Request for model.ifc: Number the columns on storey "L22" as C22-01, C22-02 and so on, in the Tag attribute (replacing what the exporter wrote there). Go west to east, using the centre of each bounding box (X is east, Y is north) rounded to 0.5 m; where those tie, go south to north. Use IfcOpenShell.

First a look at what the model holds.

```python
import ifcopenshell
import ifcopenshell.util.element
import ifcopenshell.util.placement

model = ifcopenshell.open("model.ifc")
print(model.schema)
storey = next(s for s in model.by_type("IfcBuildingStorey") if s.Name == "L22")
columns = [e for e in ifcopenshell.util.element.get_decomposition(storey) if e.is_a("IfcColumn")]
for e in sorted(columns, key=lambda e: e.id()):
    origin = ifcopenshell.util.placement.get_local_placement(e.ObjectPlacement)[:3, 3]
    print(e.id(), e.Tag, e.Name, origin.round(2) + 0.0, sep=" | ")
```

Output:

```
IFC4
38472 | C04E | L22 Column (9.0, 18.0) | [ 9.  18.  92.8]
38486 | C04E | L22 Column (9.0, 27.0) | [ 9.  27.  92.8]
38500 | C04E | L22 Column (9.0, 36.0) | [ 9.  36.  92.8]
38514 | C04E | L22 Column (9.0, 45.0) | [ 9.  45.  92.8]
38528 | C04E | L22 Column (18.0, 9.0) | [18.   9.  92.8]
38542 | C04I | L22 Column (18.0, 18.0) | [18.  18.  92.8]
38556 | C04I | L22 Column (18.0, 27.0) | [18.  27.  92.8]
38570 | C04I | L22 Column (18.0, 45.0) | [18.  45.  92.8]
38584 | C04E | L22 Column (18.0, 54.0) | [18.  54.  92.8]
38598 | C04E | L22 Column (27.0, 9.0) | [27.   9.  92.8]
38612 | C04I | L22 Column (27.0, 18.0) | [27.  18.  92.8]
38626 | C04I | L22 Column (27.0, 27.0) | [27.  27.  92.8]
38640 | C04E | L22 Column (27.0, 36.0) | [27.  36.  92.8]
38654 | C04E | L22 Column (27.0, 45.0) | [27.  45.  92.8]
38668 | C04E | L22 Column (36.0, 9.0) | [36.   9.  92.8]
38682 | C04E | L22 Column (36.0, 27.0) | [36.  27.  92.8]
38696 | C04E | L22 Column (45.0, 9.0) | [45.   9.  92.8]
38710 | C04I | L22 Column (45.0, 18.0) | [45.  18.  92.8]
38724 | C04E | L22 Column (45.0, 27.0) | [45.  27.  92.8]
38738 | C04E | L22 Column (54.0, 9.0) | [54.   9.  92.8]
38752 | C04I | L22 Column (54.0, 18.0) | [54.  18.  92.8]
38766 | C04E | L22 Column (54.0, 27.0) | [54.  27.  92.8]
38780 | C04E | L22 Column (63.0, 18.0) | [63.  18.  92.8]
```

```python
import ifcopenshell
import ifcopenshell.geom
import ifcopenshell.util.element
import ifcopenshell.util.shape

model = ifcopenshell.open("model.ifc")
settings = ifcopenshell.geom.settings()
settings.set("use-world-coords", True)


def centre(element):
    shape = ifcopenshell.geom.create_shape(settings, element)
    return ifcopenshell.util.shape.get_bbox_centroid(shape.geometry)


storey = next(s for s in model.by_type("IfcBuildingStorey") if s.Name == "L22")
columns = [e for e in ifcopenshell.util.element.get_decomposition(storey) if e.is_a("IfcColumn")]

# Insertion points can sit at a corner or the storey origin, so sort by the geometry (in metres).
centres = {e: centre(e) for e in columns}
columns.sort(key=lambda e: (round(centres[e][0] / 0.5), centres[e][1]))

for i, e in enumerate(columns, start=1):
    number = f"C22-{i:02d}"
    e.Tag = number
    print(e.id(), number)

model.write("model_rev.ifc")
```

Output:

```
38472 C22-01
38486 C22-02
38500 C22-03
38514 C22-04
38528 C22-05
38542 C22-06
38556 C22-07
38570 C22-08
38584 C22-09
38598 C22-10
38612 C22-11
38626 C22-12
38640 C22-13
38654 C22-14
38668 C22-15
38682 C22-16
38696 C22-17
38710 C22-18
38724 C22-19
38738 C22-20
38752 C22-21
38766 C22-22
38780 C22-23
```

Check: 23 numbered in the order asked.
